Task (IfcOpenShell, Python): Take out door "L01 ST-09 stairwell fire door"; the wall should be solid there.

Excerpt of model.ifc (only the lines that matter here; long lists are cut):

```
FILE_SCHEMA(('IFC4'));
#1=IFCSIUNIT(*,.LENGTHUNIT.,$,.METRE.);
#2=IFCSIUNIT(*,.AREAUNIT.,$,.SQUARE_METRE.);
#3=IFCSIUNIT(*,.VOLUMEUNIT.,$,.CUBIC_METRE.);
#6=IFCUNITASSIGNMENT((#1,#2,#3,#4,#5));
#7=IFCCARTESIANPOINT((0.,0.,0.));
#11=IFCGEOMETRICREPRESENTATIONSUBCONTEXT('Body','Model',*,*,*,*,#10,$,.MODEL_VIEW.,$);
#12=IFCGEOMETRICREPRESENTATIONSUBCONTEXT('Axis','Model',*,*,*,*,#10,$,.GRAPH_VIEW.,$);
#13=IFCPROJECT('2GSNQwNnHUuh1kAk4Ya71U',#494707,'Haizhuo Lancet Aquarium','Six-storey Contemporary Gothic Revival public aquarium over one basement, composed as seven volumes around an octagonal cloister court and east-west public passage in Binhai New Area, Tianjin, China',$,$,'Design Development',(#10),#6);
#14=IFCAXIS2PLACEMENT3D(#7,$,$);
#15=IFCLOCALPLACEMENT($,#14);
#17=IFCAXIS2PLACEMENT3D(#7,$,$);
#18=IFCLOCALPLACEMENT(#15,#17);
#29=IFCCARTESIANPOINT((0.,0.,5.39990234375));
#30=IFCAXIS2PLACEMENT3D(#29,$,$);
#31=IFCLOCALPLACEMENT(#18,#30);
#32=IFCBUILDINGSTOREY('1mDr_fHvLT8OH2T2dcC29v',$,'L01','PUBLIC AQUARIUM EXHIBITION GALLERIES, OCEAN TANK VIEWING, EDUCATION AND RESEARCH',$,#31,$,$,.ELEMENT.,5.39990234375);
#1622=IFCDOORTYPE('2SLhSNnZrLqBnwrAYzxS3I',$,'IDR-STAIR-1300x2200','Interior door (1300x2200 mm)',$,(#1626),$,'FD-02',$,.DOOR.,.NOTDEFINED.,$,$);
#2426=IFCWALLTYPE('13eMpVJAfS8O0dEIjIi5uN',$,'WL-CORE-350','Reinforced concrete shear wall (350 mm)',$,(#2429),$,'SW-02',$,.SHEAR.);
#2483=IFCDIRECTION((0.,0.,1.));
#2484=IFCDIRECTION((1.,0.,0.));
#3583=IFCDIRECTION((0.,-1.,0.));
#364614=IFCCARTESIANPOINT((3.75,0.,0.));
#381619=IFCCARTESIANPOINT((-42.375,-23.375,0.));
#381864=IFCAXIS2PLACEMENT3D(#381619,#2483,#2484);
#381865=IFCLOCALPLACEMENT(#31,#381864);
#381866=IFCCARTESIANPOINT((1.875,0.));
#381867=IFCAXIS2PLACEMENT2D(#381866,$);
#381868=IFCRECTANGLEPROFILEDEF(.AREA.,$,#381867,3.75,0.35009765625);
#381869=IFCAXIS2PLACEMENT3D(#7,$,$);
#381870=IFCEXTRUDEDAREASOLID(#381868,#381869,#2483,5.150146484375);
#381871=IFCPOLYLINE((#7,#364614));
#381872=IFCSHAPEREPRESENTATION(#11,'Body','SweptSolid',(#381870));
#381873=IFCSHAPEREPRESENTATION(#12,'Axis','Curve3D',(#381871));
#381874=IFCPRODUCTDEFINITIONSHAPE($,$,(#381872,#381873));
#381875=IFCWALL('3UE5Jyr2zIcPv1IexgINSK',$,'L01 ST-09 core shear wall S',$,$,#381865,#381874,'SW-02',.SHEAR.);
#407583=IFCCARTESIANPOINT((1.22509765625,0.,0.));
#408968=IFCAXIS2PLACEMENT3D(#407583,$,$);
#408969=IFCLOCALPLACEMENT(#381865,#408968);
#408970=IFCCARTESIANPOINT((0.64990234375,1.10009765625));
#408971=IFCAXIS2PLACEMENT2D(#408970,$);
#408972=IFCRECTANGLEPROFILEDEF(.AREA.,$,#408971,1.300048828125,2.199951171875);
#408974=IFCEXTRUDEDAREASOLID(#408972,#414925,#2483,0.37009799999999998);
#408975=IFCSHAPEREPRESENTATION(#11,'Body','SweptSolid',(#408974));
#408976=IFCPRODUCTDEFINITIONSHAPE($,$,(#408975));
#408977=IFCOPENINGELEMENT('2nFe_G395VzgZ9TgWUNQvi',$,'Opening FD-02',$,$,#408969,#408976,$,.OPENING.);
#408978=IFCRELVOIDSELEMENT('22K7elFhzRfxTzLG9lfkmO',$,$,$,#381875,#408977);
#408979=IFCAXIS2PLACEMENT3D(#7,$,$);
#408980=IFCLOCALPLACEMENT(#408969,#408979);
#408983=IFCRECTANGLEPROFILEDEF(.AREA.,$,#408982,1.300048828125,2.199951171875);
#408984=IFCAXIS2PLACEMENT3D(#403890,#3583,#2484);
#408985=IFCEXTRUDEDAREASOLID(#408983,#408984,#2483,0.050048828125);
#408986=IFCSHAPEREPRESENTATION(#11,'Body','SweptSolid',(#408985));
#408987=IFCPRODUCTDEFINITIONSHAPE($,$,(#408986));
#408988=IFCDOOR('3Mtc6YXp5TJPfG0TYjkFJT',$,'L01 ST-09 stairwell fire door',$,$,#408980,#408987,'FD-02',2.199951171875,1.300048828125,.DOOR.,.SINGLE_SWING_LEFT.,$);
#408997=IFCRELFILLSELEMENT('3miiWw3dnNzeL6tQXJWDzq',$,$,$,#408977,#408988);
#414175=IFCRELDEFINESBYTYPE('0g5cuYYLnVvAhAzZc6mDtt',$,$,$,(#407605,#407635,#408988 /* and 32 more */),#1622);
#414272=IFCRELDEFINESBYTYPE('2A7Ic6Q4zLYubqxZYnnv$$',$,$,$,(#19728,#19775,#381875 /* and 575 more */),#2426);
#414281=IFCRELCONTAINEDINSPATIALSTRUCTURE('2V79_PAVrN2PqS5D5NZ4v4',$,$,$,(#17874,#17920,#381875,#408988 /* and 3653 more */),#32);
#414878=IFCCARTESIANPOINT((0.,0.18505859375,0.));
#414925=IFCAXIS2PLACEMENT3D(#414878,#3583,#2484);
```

```python
import ifcopenshell
import ifcopenshell.api.feature
import ifcopenshell.api.root
import ifcopenshell.geom
import ifcopenshell.util.shape

model = ifcopenshell.open("model.ifc")
settings = ifcopenshell.geom.settings()


def volume(element):
    """Net volume in cubic metres, openings subtracted."""
    shape = ifcopenshell.geom.create_shape(settings, element)
    return ifcopenshell.util.shape.get_volume(shape.geometry)


door = model.by_id(408988)
opening = door.FillsVoids[0].RelatingOpeningElement
wall = opening.VoidsElements[0].RelatingBuildingElement
before = volume(wall)

ifcopenshell.api.root.remove_product(model, product=door)
ifcopenshell.api.feature.remove_feature(model, feature=opening)

after = volume(wall)

print(f"wall volume {before:.3f} -> {after:.3f} m3")

model.write("model_edited.ifc")
```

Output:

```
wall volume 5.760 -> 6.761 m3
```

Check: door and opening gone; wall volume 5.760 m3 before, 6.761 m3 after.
